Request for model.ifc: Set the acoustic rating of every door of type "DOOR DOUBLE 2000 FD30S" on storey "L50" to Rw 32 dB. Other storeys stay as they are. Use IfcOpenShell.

First a look at what the model holds.

```python
import ifcopenshell
import ifcopenshell.util.element

model = ifcopenshell.open("model.ifc")
print(model.schema)
storey = next(s for s in model.by_type("IfcBuildingStorey") if s.Name == "L50")
doors = [e for e in ifcopenshell.util.element.get_decomposition(storey) if e.is_a("IfcDoor")]
seen = {}
for e in doors:
    element_type = ifcopenshell.util.element.get_type(e)
    key = (element_type.Name if element_type != e and element_type else None, ifcopenshell.util.element.get_pset(e, "Pset_DoorCommon", "AcousticRating"))
    seen[key] = seen.get(key, 0) + 1
for (name, value), count in sorted(seen.items(), key=str):
    print(count, "x", name, "|", value)
```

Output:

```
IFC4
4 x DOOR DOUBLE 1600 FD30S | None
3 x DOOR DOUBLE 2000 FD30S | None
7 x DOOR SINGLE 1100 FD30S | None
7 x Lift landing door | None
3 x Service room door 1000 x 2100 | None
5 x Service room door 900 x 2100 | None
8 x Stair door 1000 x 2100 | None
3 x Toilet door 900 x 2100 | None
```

```python
import ifcopenshell
import ifcopenshell.api.pset
import ifcopenshell.util.element

model = ifcopenshell.open("model.ifc")

storey = next(s for s in model.by_type("IfcBuildingStorey") if s.Name == "L50")
doors = [e for e in ifcopenshell.util.element.get_decomposition(storey) if e.is_a("IfcDoor")]

count = 0
for e in doors:
    element_type = ifcopenshell.util.element.get_type(e)
    if element_type in (None, e) or element_type.Name != "DOOR DOUBLE 2000 FD30S":
        continue
    found = ifcopenshell.util.element.get_pset(e, "Pset_DoorCommon", should_inherit=False)
    if found:
        pset = model.by_id(found["id"])
        if len(ifcopenshell.util.element.get_elements_by_pset(pset)) > 1:
            pset = ifcopenshell.api.pset.unshare_pset(model, products=[e], pset=pset)[0]
    else:
        pset = ifcopenshell.api.pset.add_pset(model, product=e, name="Pset_DoorCommon")
    ifcopenshell.api.pset.edit_pset(model, pset=pset, properties={"AcousticRating": "Rw 32 dB"})
    count += 1

print(count, "doors updated")

model.write("model_updated.ifc")
```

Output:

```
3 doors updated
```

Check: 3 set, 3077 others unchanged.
